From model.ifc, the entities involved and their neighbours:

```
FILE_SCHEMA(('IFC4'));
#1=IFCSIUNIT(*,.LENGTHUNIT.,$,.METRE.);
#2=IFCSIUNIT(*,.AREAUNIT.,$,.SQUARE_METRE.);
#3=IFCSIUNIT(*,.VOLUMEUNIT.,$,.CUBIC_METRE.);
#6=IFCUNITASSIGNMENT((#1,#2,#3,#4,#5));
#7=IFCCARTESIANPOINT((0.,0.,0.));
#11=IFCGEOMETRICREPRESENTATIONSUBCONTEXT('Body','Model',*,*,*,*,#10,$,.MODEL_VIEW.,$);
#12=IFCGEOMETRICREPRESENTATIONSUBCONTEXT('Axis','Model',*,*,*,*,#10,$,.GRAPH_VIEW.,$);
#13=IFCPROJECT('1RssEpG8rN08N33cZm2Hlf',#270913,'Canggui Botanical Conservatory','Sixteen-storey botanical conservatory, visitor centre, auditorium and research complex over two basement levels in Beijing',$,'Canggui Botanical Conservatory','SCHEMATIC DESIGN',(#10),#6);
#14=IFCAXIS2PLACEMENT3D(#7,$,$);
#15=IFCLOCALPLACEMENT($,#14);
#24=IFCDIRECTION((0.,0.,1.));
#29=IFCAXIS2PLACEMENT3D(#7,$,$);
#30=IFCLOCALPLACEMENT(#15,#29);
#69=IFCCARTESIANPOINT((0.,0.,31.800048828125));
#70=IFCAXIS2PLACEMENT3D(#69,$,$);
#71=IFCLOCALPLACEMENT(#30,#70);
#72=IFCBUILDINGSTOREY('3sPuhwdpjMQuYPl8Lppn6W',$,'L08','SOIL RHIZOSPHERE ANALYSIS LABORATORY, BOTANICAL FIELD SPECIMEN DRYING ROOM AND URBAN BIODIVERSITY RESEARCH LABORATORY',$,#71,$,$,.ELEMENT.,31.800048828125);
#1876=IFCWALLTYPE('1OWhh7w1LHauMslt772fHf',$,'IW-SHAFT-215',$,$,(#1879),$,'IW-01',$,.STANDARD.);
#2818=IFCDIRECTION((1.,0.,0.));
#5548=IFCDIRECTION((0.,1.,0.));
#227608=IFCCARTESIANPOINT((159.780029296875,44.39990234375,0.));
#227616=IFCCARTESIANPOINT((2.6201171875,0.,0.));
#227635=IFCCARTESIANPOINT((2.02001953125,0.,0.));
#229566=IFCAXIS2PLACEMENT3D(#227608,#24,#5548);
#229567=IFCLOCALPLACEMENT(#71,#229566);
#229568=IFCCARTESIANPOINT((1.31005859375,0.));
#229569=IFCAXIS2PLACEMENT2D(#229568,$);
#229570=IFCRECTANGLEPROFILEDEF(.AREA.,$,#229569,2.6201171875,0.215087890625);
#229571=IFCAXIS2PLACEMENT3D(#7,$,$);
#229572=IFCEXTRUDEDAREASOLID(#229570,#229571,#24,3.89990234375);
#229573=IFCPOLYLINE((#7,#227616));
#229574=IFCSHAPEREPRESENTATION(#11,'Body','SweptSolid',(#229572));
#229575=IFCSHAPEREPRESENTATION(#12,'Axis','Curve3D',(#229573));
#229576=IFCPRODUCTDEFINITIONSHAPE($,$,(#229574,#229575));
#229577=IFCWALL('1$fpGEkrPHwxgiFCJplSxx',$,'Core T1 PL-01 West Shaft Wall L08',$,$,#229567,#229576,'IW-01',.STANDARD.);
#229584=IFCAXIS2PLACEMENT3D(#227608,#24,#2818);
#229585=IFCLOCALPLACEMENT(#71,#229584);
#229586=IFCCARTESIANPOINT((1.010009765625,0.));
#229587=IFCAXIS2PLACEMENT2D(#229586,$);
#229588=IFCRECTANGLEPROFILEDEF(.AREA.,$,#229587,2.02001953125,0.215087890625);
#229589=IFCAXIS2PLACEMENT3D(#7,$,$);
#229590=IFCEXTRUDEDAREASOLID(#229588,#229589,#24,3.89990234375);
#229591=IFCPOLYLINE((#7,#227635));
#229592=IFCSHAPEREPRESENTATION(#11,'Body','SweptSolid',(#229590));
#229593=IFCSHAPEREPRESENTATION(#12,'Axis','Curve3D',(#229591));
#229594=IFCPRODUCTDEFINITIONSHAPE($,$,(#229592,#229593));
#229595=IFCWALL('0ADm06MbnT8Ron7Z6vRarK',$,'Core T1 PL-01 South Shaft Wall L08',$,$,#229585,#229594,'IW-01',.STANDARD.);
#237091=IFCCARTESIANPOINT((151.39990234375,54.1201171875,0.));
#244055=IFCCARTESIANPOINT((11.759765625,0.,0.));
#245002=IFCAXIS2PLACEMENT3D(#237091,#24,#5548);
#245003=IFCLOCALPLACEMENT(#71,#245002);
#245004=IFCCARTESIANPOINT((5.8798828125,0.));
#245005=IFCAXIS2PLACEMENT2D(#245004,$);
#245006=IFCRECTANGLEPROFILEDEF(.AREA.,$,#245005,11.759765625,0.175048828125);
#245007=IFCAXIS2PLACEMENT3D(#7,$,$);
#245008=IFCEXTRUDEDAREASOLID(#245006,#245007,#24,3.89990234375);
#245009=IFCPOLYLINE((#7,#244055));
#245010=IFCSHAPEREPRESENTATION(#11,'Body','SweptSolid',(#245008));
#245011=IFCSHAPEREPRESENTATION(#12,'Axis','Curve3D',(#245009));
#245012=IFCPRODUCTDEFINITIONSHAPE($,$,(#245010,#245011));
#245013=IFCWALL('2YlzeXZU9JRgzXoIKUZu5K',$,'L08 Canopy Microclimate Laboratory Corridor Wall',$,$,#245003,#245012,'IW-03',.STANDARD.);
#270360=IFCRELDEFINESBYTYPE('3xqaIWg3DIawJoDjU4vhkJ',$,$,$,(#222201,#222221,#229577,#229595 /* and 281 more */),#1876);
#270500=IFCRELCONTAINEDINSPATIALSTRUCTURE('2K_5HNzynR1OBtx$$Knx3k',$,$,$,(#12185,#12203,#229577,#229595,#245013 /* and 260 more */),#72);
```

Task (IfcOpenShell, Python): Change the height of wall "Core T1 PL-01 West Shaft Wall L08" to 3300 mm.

```python
import ifcopenshell
import ifcopenshell.geom
import ifcopenshell.util.representation
import ifcopenshell.util.shape

model = ifcopenshell.open("model.ifc")
settings = ifcopenshell.geom.settings()


def volume(element):
    """Net volume in cubic metres, openings subtracted."""
    shape = ifcopenshell.geom.create_shape(settings, element)
    return ifcopenshell.util.shape.get_volume(shape.geometry)


wall = model.by_id(229577)
before = volume(wall)

body = ifcopenshell.util.representation.get_representation(wall, "Model", "Body")
solid = body.Items[0]
old_height = solid.Depth
solid.Depth = 3.3
after = volume(wall)

print(f"height {old_height:g} -> {solid.Depth:g}, volume {before:.3f} -> {after:.3f} m3")

model.write("model_updated.ifc")
```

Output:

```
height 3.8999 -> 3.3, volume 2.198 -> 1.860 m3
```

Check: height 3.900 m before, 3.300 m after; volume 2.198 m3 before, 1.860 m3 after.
